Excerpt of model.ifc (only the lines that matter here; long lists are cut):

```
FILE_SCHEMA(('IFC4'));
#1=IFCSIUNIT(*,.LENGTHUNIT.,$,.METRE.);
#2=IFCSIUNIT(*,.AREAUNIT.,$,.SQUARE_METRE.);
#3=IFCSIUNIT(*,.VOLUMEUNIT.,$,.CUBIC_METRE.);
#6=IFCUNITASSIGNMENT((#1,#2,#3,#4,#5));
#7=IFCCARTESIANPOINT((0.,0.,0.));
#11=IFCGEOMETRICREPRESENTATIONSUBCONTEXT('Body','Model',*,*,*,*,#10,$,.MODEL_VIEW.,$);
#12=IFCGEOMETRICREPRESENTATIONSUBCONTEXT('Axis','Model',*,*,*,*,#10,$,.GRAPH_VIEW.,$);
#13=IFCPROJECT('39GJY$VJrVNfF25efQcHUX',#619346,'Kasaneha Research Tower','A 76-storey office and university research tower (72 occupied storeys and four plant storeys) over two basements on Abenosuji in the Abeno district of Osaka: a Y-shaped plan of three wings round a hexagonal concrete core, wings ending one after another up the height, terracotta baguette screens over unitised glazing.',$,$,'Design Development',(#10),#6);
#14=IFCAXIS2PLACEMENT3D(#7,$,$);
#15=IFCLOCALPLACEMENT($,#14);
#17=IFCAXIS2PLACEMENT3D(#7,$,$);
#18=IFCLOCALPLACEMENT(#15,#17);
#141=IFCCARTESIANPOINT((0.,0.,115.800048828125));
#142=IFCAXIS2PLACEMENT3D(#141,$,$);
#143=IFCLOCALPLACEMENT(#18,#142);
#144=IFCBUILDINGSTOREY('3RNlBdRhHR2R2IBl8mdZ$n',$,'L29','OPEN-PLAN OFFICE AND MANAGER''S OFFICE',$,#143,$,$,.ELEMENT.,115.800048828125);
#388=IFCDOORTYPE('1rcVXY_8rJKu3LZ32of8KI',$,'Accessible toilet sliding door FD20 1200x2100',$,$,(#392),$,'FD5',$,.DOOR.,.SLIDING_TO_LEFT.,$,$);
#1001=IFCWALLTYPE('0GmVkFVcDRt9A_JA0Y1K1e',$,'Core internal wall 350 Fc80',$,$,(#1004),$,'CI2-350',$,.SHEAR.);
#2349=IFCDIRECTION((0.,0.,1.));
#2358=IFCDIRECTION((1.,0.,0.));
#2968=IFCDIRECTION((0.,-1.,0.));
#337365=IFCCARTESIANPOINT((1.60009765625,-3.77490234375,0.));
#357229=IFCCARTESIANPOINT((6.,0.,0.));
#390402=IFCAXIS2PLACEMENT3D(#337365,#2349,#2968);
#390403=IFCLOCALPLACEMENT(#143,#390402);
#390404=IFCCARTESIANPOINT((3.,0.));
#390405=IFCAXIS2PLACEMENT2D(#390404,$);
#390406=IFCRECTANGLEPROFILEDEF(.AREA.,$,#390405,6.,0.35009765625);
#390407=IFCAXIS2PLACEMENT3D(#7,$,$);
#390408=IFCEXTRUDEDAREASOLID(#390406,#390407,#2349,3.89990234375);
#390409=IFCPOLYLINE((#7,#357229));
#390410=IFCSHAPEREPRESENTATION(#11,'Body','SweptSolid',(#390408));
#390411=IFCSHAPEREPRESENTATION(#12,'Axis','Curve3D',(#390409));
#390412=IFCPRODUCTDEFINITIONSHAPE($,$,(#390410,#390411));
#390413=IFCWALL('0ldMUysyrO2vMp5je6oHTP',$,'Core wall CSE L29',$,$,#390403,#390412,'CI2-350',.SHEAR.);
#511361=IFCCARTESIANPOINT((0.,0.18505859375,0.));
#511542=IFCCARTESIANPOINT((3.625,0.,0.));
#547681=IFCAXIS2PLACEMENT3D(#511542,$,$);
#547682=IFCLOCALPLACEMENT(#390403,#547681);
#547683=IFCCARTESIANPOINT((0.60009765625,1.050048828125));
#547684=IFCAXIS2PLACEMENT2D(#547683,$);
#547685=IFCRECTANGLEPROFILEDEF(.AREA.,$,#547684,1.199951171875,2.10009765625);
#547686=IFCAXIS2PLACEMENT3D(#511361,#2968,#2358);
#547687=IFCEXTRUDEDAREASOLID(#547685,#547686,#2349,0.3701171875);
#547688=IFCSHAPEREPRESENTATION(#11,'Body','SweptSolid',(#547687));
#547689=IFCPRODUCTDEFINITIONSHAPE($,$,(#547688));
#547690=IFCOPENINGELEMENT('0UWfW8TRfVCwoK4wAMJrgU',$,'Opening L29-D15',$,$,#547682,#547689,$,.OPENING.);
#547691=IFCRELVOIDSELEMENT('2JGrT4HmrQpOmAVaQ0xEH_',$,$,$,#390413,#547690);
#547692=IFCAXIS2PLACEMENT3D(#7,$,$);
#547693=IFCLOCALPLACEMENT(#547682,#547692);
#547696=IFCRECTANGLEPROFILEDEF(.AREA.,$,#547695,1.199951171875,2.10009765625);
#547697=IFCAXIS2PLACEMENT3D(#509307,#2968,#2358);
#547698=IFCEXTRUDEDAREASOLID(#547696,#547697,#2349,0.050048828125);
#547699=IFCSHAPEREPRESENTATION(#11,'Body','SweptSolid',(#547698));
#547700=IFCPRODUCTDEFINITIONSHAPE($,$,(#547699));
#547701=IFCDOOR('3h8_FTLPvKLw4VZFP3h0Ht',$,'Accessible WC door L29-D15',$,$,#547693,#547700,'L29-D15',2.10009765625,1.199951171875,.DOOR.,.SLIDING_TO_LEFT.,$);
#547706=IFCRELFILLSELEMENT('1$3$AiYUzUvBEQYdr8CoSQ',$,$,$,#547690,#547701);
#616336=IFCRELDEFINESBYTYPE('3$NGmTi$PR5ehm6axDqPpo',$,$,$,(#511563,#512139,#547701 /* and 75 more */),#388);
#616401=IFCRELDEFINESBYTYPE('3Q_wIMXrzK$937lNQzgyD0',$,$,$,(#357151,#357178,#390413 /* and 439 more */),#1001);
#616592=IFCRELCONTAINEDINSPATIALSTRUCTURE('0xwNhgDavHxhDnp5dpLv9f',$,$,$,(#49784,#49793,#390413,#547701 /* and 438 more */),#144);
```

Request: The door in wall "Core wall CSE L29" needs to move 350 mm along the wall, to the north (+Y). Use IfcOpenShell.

```python
import ifcopenshell
import ifcopenshell.api.geometry
import ifcopenshell.util.placement
import ifcopenshell.util.unit

model = ifcopenshell.open("model.ifc")
unit_scale = ifcopenshell.util.unit.calculate_unit_scale(model)

door = model.by_guid("3h8_FTLPvKLw4VZFP3h0Ht")
opening = door.FillsVoids[0].RelatingOpeningElement
wall = opening.VoidsElements[0].RelatingBuildingElement

wall_matrix = ifcopenshell.util.placement.get_local_placement(wall.ObjectPlacement)
shift = wall_matrix[:3, 0] * -0.35 / unit_scale
before = ifcopenshell.util.placement.get_local_placement(door.ObjectPlacement)[:3, 3].copy()

# The door is placed relative to its opening, so it follows when the opening moves.
matrix = ifcopenshell.util.placement.get_local_placement(opening.ObjectPlacement)
matrix[:3, 3] += shift
ifcopenshell.api.geometry.edit_object_placement(
    model, product=opening, matrix=matrix, is_si=False, should_transform_children=True
)

after = ifcopenshell.util.placement.get_local_placement(door.ObjectPlacement)[:3, 3]
print("door moved by", (after - before).round(3) + 0.0)

model.write("model-out.ifc")
```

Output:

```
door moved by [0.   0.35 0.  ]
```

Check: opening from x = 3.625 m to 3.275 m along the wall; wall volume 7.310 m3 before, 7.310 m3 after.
